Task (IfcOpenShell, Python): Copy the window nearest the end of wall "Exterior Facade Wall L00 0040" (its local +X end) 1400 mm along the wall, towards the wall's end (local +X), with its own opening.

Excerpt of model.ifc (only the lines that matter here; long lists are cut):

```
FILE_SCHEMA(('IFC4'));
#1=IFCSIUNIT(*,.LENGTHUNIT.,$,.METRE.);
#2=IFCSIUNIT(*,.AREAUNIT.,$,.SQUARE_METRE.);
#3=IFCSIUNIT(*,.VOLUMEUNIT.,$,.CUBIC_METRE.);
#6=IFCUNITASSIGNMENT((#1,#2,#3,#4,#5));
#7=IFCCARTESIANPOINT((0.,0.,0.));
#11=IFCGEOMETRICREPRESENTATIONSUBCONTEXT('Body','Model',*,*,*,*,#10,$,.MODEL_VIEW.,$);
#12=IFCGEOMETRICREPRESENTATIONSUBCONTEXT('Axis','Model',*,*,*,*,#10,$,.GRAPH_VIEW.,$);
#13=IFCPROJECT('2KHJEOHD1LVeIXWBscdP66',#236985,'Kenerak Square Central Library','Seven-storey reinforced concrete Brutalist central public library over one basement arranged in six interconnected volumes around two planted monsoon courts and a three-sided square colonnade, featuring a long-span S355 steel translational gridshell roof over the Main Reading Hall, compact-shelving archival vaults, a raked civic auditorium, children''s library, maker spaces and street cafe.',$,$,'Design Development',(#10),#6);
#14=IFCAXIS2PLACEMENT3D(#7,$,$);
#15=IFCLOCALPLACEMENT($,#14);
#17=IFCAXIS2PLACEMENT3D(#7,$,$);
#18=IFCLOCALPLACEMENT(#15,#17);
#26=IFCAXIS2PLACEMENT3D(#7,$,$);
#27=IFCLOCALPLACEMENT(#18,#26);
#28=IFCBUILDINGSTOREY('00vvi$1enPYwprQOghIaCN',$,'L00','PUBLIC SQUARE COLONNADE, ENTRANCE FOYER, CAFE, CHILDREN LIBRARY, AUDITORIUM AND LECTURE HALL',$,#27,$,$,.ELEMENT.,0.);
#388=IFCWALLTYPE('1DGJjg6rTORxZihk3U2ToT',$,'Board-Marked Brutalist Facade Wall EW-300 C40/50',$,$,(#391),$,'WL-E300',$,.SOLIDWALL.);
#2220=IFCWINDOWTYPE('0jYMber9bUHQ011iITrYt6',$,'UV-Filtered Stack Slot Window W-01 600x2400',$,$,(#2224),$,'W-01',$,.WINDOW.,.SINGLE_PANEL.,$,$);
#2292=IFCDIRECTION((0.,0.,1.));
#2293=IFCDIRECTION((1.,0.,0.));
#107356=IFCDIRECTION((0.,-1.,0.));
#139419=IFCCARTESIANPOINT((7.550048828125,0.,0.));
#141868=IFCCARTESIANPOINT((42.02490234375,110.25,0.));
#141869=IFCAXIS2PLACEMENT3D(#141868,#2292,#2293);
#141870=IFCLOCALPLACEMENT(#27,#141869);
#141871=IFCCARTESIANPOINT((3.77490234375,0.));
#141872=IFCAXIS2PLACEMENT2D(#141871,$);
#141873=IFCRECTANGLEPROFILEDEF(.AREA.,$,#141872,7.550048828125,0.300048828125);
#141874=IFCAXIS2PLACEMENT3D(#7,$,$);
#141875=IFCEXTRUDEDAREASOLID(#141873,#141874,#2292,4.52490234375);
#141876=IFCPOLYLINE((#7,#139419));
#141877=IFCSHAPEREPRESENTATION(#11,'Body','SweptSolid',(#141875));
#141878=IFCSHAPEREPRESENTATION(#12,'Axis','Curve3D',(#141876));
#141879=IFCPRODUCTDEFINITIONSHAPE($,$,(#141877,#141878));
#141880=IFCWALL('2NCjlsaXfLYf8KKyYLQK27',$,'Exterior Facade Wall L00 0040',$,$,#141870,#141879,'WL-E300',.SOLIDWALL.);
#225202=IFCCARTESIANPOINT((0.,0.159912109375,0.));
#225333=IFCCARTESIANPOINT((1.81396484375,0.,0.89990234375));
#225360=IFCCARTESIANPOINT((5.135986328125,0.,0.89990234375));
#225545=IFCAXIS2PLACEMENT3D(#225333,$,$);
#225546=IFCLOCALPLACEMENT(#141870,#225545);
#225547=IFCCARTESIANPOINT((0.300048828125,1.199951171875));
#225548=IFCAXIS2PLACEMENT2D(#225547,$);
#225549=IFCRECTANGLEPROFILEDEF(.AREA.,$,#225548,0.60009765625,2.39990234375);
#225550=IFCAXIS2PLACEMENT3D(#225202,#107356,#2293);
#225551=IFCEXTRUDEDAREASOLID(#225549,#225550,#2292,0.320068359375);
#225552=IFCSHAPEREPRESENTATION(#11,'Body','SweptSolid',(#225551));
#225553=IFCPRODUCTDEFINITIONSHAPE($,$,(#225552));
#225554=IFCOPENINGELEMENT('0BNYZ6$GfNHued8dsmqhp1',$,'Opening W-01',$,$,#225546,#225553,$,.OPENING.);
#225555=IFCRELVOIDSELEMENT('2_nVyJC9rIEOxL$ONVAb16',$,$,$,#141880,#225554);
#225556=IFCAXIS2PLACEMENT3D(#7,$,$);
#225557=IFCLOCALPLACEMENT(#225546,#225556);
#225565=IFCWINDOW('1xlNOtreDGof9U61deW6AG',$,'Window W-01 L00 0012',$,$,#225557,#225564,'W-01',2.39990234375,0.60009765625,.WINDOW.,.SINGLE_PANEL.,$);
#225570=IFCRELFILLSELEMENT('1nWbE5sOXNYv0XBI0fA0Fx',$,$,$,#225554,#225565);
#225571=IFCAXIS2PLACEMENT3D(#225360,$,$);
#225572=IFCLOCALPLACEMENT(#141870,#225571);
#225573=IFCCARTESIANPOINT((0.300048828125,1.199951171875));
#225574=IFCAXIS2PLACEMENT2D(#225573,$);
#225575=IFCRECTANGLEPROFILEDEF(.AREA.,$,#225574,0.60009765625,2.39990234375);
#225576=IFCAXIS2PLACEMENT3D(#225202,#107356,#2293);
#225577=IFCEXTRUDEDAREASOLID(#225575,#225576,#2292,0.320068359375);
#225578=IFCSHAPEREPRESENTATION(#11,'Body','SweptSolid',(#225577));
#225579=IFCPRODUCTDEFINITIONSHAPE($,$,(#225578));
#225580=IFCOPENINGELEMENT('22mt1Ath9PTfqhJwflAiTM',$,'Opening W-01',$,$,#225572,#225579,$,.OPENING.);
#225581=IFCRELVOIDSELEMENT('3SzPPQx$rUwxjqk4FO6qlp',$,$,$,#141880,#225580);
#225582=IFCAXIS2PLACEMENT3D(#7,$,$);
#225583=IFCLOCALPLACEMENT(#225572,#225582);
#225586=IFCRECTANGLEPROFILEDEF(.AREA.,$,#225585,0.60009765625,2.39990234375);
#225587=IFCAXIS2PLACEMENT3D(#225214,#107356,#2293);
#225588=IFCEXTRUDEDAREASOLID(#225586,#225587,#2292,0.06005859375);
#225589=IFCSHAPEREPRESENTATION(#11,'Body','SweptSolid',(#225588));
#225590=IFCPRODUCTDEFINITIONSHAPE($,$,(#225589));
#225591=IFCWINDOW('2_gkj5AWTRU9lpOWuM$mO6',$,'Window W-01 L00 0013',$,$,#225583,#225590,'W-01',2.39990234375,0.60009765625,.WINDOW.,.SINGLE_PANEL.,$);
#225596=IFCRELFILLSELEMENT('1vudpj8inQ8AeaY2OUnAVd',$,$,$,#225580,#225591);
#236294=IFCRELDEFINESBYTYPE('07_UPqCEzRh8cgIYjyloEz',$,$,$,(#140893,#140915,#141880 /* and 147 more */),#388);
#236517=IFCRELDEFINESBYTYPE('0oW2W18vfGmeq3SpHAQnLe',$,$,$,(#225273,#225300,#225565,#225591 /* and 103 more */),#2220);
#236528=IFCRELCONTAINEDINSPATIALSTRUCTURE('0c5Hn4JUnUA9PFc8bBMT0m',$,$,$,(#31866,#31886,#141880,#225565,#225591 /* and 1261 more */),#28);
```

```python
import ifcopenshell
import ifcopenshell.api.feature
import ifcopenshell.api.geometry
import ifcopenshell.api.root
import ifcopenshell.geom
import ifcopenshell.util.element
import ifcopenshell.util.placement
import ifcopenshell.util.shape
import ifcopenshell.util.unit

model = ifcopenshell.open("model.ifc")
unit_scale = ifcopenshell.util.unit.calculate_unit_scale(model)
settings = ifcopenshell.geom.settings()


def volume(element):
    """Net volume in cubic metres, openings subtracted."""
    shape = ifcopenshell.geom.create_shape(settings, element)
    return ifcopenshell.util.shape.get_volume(shape.geometry)


window = model.by_guid("2_gkj5AWTRU9lpOWuM$mO6")
opening = window.FillsVoids[0].RelatingOpeningElement
wall = opening.VoidsElements[0].RelatingBuildingElement
before = volume(wall)
shift = ifcopenshell.util.placement.get_local_placement(wall.ObjectPlacement)[:3, 0] * 1.4 / unit_scale

# copy_class copies the void relationship, type, container and properties, but no geometry.
new_opening = ifcopenshell.api.root.copy_class(model, product=opening)
new_opening.Representation = ifcopenshell.util.element.copy_deep(
    model, opening.Representation, exclude=["IfcGeometricRepresentationContext", "IfcRepresentationMap"]
)
new_window = ifcopenshell.api.root.copy_class(model, product=window)
new_window.Representation = ifcopenshell.util.element.copy_deep(
    model, window.Representation, exclude=["IfcGeometricRepresentationContext", "IfcRepresentationMap"]
)
new_window.Tag = None
ifcopenshell.api.feature.add_filling(model, opening=new_opening, element=new_window)

for old, new in ((opening, new_opening), (window, new_window)):
    matrix = ifcopenshell.util.placement.get_local_placement(old.ObjectPlacement)
    matrix[:3, 3] += shift
    ifcopenshell.api.geometry.edit_object_placement(model, product=new, matrix=matrix, is_si=False)

after = volume(wall)

print(f"wall volume {before:.3f} -> {after:.3f} m3")

model.write("model_v2.ifc")
```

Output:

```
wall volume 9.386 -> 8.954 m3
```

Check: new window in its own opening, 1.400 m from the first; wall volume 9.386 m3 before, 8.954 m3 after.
